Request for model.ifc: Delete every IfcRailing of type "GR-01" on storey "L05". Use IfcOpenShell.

First a look at what the model holds.

```python
import ifcopenshell
import ifcopenshell.util.element

model = ifcopenshell.open("model.ifc")
print(model.schema)
storey = next(s for s in model.by_type("IfcBuildingStorey") if s.Name == "L05")
railings = [e for e in ifcopenshell.util.element.get_decomposition(storey) if e.is_a("IfcRailing")]
seen = {}
for e in railings:
    element_type = ifcopenshell.util.element.get_type(e)
    name = element_type.Name if element_type not in (None, e) else None
    seen[name] = seen.get(name, 0) + 1
for name, count in sorted(seen.items(), key=str):
    print(count, "x", name)
```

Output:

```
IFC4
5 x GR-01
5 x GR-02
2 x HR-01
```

```python
import ifcopenshell
import ifcopenshell.api.root
import ifcopenshell.util.element

model = ifcopenshell.open("model.ifc")

storey = next(s for s in model.by_type("IfcBuildingStorey") if s.Name == "L05")
railings = [e for e in ifcopenshell.util.element.get_decomposition(storey) if e.is_a("IfcRailing")]
targets = [e for e in railings if (t := ifcopenshell.util.element.get_type(e)) not in (None, e) and t.Name == "GR-01"]

for e in targets:
    ifcopenshell.api.root.remove_product(model, product=e)
print(len(targets), "removed")

model.write("model_updated.ifc")
```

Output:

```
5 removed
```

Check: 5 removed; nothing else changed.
